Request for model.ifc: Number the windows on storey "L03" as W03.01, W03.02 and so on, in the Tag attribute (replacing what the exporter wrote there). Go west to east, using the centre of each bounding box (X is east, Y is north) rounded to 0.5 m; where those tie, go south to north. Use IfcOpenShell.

First a look at what the model holds.

```python
import ifcopenshell
import ifcopenshell.util.element
import ifcopenshell.util.placement

model = ifcopenshell.open("model.ifc")
print(model.schema)
storey = next(s for s in model.by_type("IfcBuildingStorey") if s.Name == "L03")
windows = [e for e in ifcopenshell.util.element.get_decomposition(storey) if e.is_a("IfcWindow")]
for e in sorted(windows, key=lambda e: e.id()):
    origin = ifcopenshell.util.placement.get_local_placement(e.ObjectPlacement)[:3, 3]
    print(e.id(), e.Tag, e.Name, origin.round(2) + 0.0, sep=" | ")
```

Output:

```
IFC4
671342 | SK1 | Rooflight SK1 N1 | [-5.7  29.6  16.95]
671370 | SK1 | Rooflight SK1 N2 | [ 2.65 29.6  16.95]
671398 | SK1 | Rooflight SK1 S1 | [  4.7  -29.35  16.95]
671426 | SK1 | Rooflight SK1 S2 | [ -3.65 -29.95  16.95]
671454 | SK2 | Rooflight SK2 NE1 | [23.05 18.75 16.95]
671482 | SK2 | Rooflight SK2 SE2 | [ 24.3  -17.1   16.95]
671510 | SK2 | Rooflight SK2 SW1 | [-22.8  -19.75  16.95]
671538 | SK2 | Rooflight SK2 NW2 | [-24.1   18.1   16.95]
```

```python
import ifcopenshell
import ifcopenshell.geom
import ifcopenshell.util.element
import ifcopenshell.util.shape

model = ifcopenshell.open("model.ifc")
settings = ifcopenshell.geom.settings()
settings.set("use-world-coords", True)


def centre(element):
    shape = ifcopenshell.geom.create_shape(settings, element)
    return ifcopenshell.util.shape.get_bbox_centroid(shape.geometry)


storey = next(s for s in model.by_type("IfcBuildingStorey") if s.Name == "L03")
windows = [e for e in ifcopenshell.util.element.get_decomposition(storey) if e.is_a("IfcWindow")]

# Insertion points can sit at a corner or the storey origin, so sort by the geometry (in metres).
centres = {e: centre(e) for e in windows}
windows.sort(key=lambda e: (round(centres[e][0] / 0.5), centres[e][1]))

for i, e in enumerate(windows, start=1):
    number = f"W03.{i:02d}"
    e.Tag = number
    print(e.id(), number)

model.write("model_updated.ifc")
```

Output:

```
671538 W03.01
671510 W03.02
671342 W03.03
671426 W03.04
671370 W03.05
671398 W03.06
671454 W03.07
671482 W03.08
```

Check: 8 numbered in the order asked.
